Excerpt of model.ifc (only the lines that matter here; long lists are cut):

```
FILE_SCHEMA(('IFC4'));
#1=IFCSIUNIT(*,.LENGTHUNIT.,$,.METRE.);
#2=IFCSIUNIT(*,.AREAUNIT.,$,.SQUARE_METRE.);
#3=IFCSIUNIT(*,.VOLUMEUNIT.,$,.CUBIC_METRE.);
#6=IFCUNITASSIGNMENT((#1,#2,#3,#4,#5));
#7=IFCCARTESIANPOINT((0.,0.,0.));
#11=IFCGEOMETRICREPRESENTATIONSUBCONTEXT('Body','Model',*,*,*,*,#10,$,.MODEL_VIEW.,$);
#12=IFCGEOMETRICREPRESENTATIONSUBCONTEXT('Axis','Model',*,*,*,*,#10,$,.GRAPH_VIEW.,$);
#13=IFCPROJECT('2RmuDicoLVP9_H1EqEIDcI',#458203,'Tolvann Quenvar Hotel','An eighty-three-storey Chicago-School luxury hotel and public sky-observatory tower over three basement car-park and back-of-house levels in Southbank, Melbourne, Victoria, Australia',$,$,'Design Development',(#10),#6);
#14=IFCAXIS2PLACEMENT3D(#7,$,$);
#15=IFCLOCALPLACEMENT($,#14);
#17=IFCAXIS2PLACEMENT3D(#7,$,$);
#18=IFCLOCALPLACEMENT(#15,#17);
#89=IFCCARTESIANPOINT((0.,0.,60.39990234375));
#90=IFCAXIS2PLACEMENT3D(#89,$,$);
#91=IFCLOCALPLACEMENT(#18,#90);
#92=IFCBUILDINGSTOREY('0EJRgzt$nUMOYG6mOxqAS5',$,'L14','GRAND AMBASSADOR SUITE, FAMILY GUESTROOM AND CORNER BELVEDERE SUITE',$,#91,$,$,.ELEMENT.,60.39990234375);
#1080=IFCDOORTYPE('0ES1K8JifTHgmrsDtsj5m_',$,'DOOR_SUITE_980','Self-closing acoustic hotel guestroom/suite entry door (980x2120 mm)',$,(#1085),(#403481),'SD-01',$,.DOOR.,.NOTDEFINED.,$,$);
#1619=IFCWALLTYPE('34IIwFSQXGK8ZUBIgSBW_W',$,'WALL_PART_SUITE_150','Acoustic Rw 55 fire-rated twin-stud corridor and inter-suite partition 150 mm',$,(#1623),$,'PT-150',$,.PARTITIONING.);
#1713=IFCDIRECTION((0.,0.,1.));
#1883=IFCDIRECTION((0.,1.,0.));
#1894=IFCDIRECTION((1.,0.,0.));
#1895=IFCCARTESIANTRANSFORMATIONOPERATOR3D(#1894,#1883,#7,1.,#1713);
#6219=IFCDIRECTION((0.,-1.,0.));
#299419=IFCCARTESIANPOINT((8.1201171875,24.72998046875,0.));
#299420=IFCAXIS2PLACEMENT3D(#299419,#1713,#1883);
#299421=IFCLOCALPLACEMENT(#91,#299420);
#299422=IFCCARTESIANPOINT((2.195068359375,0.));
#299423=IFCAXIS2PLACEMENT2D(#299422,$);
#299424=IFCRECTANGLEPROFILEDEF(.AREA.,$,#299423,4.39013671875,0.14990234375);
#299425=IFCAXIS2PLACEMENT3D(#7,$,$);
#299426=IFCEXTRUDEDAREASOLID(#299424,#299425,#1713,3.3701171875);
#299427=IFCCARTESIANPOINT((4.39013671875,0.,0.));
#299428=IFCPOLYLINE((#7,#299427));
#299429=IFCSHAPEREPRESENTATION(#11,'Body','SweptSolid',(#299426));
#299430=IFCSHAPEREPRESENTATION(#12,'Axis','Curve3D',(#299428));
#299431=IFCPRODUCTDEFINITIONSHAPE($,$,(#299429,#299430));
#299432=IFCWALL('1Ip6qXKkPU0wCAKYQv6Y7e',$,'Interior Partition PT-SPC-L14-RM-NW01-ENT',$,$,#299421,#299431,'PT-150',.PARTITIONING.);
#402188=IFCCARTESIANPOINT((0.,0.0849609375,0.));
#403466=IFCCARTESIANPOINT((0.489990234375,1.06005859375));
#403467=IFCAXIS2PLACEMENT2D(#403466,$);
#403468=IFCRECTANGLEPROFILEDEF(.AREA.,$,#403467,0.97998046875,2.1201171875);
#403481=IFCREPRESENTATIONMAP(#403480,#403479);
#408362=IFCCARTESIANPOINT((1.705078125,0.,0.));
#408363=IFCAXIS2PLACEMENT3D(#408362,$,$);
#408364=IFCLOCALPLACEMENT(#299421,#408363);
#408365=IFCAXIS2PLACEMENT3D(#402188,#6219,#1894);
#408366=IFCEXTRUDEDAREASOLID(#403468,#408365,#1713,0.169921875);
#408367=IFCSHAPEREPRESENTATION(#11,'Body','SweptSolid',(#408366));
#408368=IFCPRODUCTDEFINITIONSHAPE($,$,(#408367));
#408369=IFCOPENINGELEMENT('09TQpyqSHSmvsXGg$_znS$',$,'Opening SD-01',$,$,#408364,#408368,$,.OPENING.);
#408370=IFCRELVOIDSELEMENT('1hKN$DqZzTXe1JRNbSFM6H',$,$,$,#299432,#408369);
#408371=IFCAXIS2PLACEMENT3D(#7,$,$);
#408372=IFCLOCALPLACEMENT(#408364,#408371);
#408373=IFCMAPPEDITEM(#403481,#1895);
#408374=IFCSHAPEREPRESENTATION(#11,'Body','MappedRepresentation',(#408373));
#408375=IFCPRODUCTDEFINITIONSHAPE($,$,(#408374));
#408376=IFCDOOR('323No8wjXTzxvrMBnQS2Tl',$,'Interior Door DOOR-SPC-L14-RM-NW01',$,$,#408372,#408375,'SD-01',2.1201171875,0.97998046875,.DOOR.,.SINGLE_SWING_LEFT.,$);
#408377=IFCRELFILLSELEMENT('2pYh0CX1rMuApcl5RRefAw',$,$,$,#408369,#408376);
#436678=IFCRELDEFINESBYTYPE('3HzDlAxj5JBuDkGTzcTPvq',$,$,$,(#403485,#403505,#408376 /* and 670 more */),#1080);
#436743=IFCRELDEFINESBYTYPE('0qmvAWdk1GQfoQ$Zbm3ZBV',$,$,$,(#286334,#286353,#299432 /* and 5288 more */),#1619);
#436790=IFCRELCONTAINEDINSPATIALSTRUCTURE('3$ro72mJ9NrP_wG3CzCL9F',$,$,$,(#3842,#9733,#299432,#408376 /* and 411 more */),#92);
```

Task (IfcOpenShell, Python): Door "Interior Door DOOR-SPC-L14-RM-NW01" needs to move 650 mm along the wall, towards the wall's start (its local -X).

```python
import ifcopenshell
import ifcopenshell.api.geometry
import ifcopenshell.util.placement

model = ifcopenshell.open("model.ifc")

door = model.by_guid("323No8wjXTzxvrMBnQS2Tl")
opening = door.FillsVoids[0].RelatingOpeningElement
wall = opening.VoidsElements[0].RelatingBuildingElement

wall_matrix = ifcopenshell.util.placement.get_local_placement(wall.ObjectPlacement)
shift = wall_matrix[:3, 0] * -0.65
before = ifcopenshell.util.placement.get_local_placement(door.ObjectPlacement)[:3, 3].copy()

# The door is placed relative to its opening, so it follows when the opening moves.
matrix = ifcopenshell.util.placement.get_local_placement(opening.ObjectPlacement)
matrix[:3, 3] += shift
ifcopenshell.api.geometry.edit_object_placement(
    model, product=opening, matrix=matrix, is_si=False, should_transform_children=True
)

after = ifcopenshell.util.placement.get_local_placement(door.ObjectPlacement)[:3, 3]
print("door moved by", (after - before).round(3) + 0.0)

model.write("model_edited.ifc")
```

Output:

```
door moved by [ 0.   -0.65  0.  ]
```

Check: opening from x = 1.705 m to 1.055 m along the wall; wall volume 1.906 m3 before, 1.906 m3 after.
